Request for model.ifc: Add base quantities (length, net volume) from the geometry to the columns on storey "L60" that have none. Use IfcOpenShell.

First a look at what the model holds.

```python
import ifcopenshell
import ifcopenshell.util.element
import ifcopenshell.util.unit

model = ifcopenshell.open("model.ifc")
print(model.schema)
for unit_type in ("LENGTHUNIT", "AREAUNIT", "VOLUMEUNIT"):
    print(unit_type, ifcopenshell.util.unit.calculate_unit_scale(model, unit_type))
storey = next(s for s in model.by_type("IfcBuildingStorey") if s.Name == "L60")
columns = [e for e in ifcopenshell.util.element.get_decomposition(storey) if e.is_a("IfcColumn")]
for e in sorted(columns, key=lambda e: e.id()):
    print(e.id(), e.is_a(), e.Name, list(ifcopenshell.util.element.get_psets(e, qtos_only=True)), sep=" | ")
```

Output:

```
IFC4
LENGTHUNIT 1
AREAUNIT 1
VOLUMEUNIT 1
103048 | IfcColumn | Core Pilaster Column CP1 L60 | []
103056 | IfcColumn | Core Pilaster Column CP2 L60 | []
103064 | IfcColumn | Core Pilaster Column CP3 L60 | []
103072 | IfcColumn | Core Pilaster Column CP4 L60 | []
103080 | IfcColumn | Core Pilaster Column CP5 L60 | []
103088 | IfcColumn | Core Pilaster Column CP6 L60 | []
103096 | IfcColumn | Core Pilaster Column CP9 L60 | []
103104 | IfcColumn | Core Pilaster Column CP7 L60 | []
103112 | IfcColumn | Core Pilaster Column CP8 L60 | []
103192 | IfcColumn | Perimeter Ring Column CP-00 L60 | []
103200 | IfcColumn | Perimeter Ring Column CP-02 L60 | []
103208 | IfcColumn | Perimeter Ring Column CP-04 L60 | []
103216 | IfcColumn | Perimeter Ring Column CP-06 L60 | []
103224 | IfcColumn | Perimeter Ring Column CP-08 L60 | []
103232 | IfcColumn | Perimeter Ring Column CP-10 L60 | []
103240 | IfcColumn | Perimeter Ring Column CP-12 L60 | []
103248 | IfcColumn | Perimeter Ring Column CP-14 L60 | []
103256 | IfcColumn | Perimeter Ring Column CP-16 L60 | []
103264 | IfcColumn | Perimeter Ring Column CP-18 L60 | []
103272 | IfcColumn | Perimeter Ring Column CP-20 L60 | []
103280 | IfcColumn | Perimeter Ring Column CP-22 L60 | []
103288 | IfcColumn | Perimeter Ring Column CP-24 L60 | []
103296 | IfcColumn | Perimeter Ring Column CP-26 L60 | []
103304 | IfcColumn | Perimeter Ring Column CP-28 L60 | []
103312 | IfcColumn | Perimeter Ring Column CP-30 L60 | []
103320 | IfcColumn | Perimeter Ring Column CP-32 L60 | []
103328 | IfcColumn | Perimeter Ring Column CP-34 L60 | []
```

```python
import ifcopenshell
import ifcopenshell.api.pset
import ifcopenshell.geom
import ifcopenshell.util.element
import ifcopenshell.util.shape
import ifcopenshell.util.unit

model = ifcopenshell.open("model.ifc")
unit_scale = ifcopenshell.util.unit.calculate_unit_scale(model)
volume_scale = ifcopenshell.util.unit.calculate_unit_scale(model, "VOLUMEUNIT")
settings = ifcopenshell.geom.settings()

storey = next(s for s in model.by_type("IfcBuildingStorey") if s.Name == "L60")
columns = [e for e in ifcopenshell.util.element.get_decomposition(storey) if e.is_a("IfcColumn")]

for e in sorted(columns, key=lambda e: e.id()):
    if ifcopenshell.util.element.get_psets(e, qtos_only=True, should_inherit=False):
        continue
    # Geometry comes back in metres, in the element's own axes.
    shape = ifcopenshell.geom.create_shape(settings, e)
    values = {
        "Length": ifcopenshell.util.shape.get_z(shape.geometry) / unit_scale,
        "NetVolume": ifcopenshell.util.shape.get_volume(shape.geometry) / volume_scale,
    }
    qto = ifcopenshell.api.pset.add_qto(model, product=e, name="Qto_ColumnBaseQuantities")
    ifcopenshell.api.pset.edit_qto(model, qto=qto, properties=values)
    print(e.id(), {k: round(v, 3) for k, v in values.items()})

model.write("model_updated.ifc")
```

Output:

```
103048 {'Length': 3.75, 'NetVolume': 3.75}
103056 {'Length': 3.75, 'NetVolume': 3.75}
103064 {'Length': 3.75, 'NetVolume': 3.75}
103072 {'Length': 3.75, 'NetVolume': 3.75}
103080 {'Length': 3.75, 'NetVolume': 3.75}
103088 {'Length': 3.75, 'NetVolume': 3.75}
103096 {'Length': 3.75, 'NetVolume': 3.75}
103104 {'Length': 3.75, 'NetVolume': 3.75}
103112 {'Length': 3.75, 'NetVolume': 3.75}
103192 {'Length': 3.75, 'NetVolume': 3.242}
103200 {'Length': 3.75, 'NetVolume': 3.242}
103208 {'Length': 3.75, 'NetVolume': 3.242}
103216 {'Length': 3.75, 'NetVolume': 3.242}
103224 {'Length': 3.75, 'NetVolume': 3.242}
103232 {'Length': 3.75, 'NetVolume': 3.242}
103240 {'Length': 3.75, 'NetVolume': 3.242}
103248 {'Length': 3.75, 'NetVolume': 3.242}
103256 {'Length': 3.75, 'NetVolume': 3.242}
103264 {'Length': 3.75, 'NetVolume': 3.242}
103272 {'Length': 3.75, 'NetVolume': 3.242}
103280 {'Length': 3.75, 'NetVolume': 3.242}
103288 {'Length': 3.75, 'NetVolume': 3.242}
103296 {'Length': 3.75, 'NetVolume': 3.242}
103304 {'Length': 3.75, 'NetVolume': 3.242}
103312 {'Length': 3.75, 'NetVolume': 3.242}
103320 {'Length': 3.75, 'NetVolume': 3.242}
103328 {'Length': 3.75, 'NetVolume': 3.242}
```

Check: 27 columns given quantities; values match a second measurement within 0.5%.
